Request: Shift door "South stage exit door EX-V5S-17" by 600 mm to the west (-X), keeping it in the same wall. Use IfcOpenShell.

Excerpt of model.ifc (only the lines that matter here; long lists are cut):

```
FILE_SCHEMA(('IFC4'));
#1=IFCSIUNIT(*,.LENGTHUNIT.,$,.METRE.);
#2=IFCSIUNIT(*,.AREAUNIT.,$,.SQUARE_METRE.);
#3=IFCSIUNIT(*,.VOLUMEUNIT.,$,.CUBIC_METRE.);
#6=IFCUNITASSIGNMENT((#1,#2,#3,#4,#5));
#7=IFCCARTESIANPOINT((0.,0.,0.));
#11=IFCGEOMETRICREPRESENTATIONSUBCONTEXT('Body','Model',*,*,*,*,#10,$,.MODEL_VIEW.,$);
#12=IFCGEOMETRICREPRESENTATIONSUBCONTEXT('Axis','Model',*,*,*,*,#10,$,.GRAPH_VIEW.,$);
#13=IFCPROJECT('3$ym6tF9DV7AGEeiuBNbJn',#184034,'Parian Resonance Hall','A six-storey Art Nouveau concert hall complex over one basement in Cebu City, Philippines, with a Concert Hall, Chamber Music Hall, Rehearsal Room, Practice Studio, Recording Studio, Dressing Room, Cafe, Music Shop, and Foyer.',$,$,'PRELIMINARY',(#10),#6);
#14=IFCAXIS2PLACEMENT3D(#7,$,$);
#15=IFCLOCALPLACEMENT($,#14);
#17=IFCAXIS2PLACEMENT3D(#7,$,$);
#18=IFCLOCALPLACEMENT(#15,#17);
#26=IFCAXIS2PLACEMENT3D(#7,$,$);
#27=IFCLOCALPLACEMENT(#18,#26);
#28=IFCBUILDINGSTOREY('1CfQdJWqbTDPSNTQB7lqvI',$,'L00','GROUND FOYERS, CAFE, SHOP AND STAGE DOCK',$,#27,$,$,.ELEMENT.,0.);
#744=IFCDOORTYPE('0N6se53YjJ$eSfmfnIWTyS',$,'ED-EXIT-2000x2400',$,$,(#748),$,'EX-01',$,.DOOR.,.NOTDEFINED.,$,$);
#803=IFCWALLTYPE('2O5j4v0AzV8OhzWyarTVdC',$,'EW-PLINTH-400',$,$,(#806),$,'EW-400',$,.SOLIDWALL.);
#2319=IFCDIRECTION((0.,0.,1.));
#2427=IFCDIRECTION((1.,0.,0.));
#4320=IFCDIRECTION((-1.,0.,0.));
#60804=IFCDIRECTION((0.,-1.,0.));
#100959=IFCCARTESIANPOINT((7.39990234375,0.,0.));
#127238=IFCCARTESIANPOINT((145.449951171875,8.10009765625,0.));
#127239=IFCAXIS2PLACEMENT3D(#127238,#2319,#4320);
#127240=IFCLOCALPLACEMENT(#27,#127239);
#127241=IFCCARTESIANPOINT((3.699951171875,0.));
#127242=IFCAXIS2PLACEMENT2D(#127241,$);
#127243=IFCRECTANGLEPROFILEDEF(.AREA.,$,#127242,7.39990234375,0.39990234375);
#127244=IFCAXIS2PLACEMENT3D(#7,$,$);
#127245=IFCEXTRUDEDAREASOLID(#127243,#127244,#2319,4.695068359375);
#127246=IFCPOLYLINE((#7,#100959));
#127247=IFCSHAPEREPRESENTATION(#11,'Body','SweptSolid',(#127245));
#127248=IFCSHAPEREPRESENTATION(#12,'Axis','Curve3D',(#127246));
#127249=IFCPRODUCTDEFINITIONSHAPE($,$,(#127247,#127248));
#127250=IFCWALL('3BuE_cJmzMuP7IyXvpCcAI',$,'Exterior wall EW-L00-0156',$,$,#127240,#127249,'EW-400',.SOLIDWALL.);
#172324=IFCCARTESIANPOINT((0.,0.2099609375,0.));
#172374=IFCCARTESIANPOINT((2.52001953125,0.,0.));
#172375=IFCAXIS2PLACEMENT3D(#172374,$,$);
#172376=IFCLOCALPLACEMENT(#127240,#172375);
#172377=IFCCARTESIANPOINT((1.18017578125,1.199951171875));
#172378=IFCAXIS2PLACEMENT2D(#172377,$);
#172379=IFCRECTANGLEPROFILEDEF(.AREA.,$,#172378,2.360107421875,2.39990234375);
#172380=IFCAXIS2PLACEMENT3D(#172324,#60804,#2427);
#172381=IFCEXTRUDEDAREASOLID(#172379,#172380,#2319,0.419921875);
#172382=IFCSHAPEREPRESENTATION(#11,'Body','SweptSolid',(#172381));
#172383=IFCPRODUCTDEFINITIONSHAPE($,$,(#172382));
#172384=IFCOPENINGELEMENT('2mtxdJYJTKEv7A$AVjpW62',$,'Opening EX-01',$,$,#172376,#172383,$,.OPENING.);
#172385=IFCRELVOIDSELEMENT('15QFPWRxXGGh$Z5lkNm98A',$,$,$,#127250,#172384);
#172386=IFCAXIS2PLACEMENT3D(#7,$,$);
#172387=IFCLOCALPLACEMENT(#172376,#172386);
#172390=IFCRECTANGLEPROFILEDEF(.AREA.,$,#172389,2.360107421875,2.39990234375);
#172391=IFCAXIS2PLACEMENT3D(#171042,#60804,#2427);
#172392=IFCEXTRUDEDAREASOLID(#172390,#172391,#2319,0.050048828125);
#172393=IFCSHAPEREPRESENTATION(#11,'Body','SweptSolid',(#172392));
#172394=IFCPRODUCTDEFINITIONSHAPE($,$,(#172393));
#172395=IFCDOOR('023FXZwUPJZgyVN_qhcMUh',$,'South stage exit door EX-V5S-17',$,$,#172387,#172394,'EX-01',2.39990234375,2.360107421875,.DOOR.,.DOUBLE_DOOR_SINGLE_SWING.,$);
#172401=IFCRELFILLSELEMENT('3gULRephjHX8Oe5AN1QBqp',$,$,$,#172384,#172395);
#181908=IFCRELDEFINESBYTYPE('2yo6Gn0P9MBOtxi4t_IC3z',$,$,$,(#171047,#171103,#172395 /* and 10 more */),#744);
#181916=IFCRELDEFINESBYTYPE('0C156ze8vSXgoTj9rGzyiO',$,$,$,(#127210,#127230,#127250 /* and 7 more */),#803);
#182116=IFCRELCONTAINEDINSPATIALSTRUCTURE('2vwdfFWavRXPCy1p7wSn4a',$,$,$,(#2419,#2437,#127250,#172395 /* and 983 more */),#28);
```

```python
import ifcopenshell
import ifcopenshell.api.geometry
import ifcopenshell.util.placement
import ifcopenshell.util.unit

model = ifcopenshell.open("model.ifc")
unit_scale = ifcopenshell.util.unit.calculate_unit_scale(model)

door = model.by_guid("023FXZwUPJZgyVN_qhcMUh")
opening = door.FillsVoids[0].RelatingOpeningElement
wall = opening.VoidsElements[0].RelatingBuildingElement

wall_matrix = ifcopenshell.util.placement.get_local_placement(wall.ObjectPlacement)
shift = wall_matrix[:3, 0] * 0.6 / unit_scale
before = ifcopenshell.util.placement.get_local_placement(door.ObjectPlacement)[:3, 3].copy()

# The door is placed relative to its opening, so it follows when the opening moves.
matrix = ifcopenshell.util.placement.get_local_placement(opening.ObjectPlacement)
matrix[:3, 3] += shift
ifcopenshell.api.geometry.edit_object_placement(
    model, product=opening, matrix=matrix, is_si=False, should_transform_children=True
)

after = ifcopenshell.util.placement.get_local_placement(door.ObjectPlacement)[:3, 3]
print("door moved by", (after - before).round(3) + 0.0)

model.write("model_updated.ifc")
```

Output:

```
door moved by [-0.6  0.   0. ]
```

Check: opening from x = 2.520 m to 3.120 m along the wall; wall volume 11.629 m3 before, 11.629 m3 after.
